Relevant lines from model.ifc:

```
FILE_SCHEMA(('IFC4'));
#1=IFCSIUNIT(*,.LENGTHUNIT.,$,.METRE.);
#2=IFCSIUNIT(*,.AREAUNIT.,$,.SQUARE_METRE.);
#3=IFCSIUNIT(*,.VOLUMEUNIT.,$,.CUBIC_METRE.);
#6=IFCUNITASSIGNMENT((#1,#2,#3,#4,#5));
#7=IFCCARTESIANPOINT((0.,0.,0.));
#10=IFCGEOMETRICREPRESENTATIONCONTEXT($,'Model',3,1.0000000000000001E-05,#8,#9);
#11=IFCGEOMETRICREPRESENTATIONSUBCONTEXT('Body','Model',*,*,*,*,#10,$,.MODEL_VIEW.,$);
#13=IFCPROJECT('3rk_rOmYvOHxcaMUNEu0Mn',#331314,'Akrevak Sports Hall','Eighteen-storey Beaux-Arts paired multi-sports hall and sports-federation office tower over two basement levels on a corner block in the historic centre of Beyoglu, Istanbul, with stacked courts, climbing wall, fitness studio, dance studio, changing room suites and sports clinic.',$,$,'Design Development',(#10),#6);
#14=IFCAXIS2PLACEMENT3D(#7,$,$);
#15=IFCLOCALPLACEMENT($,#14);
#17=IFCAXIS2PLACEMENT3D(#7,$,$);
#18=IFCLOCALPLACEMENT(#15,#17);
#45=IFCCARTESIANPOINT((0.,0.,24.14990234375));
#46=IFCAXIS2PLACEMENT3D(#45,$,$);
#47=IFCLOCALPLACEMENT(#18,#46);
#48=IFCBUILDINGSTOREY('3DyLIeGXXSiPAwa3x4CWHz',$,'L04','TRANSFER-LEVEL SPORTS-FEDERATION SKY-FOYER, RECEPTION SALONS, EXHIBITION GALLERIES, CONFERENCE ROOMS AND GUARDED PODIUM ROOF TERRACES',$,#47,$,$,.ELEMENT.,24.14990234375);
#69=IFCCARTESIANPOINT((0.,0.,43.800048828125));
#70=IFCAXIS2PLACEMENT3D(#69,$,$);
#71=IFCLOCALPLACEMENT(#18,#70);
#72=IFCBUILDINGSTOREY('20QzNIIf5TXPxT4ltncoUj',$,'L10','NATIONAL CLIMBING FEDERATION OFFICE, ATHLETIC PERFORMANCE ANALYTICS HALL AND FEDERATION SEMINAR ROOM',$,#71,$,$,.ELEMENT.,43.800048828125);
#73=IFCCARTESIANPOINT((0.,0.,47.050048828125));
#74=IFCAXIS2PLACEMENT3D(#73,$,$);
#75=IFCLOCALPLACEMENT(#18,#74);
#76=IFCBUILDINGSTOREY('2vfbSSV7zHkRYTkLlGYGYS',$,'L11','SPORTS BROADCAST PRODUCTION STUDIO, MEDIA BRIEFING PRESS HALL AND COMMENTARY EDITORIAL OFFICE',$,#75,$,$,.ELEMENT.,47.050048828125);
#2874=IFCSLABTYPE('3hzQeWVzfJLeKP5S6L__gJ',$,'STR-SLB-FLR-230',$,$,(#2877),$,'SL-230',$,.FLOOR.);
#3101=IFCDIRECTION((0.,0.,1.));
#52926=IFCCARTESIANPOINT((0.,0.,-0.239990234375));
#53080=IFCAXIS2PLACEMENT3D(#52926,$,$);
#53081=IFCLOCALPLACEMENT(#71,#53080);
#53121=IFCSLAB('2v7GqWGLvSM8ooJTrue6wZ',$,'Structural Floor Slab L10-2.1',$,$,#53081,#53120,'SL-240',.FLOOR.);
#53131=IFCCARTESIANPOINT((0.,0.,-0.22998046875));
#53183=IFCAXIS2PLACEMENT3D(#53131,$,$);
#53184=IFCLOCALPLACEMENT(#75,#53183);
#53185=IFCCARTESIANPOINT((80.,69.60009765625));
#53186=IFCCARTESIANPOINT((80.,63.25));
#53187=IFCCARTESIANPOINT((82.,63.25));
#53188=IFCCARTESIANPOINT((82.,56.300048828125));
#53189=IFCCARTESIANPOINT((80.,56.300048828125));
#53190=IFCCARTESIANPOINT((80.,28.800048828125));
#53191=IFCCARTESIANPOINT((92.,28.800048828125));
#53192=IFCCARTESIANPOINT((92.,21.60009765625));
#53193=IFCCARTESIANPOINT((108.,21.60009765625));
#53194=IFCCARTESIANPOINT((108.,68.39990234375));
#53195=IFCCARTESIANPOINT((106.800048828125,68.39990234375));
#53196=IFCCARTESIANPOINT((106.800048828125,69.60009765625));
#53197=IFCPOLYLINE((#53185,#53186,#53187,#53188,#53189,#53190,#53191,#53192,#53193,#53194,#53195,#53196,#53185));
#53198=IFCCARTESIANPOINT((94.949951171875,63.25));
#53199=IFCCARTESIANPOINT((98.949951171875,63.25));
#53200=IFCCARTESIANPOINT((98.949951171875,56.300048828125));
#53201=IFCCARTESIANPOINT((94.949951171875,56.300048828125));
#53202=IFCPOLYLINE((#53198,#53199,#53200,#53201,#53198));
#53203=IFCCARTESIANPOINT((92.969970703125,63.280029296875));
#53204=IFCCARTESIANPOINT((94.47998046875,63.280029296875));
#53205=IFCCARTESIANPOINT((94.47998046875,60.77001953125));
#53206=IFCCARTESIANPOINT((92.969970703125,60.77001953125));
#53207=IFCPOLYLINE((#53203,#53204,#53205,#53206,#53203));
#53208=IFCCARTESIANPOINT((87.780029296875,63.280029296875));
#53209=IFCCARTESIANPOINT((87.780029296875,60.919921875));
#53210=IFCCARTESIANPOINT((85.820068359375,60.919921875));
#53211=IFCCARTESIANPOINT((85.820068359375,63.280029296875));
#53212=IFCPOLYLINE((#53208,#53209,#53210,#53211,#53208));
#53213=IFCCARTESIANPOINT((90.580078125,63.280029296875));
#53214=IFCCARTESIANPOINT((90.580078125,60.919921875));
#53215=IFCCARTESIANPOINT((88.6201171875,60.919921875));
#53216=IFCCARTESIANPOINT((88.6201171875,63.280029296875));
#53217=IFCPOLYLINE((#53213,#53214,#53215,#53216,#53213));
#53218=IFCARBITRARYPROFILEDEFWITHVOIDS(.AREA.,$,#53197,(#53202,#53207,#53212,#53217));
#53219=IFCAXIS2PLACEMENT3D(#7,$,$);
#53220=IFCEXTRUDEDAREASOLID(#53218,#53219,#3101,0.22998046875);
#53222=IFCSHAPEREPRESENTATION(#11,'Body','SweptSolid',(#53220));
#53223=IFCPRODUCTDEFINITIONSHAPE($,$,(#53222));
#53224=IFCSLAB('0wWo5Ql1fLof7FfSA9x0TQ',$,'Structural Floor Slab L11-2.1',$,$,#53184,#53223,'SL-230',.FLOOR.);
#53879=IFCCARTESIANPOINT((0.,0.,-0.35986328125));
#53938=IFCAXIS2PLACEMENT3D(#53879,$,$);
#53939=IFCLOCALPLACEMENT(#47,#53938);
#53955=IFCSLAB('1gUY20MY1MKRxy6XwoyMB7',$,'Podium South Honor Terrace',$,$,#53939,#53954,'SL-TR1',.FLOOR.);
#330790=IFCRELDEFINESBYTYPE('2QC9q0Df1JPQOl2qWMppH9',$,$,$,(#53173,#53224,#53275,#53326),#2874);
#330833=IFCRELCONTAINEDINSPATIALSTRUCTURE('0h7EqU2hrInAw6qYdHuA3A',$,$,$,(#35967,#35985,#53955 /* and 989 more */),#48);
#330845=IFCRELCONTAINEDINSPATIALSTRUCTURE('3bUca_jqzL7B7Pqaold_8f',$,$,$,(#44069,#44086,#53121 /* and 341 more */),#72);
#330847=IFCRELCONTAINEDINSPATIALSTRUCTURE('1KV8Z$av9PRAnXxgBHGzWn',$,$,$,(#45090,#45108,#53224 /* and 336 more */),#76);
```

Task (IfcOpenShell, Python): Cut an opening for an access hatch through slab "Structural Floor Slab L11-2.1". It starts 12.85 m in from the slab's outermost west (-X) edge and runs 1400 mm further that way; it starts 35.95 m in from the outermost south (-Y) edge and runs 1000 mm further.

```python
import numpy as np
import ifcopenshell
import ifcopenshell.api.feature
import ifcopenshell.api.geometry
import ifcopenshell.api.root
import ifcopenshell.geom
import ifcopenshell.util.placement
import ifcopenshell.util.representation
import ifcopenshell.util.shape
import ifcopenshell.util.unit

model = ifcopenshell.open("model.ifc")
unit_scale = ifcopenshell.util.unit.calculate_unit_scale(model)
settings = ifcopenshell.geom.settings()


def volume(element):
    """Net volume in cubic metres, openings subtracted."""
    shape = ifcopenshell.geom.create_shape(settings, element)
    return ifcopenshell.util.shape.get_volume(shape.geometry)


slab = model.by_id(53224)
before = volume(slab)

# Extent in the slab's own axes, in metres. The edges named are its -X and -Y sides.
slab_shape = ifcopenshell.geom.create_shape(settings, slab)
vertices = ifcopenshell.util.shape.get_vertices(slab_shape.geometry)
x_min, y_min, bottom = vertices.min(axis=0)
top = vertices[:, 2].max()

opening = ifcopenshell.api.root.create_entity(model, ifc_class="IfcOpeningElement", name="Access hatch opening", predefined_type="OPENING")
context = ifcopenshell.util.representation.get_context(model, "Model", "Body", "MODEL_VIEW")
width, depth = 1.4, 1
outline = [(0.0, 0.0), (width, 0.0), (width, depth), (0.0, depth), (0.0, 0.0)]
# Overshoot both faces by 50 mm so the cut is clean.
shape = ifcopenshell.api.geometry.add_slab_representation(
    model, context=context, depth=top - bottom + 0.1, polyline=outline
)
ifcopenshell.api.geometry.assign_representation(model, product=opening, representation=shape)

matrix = ifcopenshell.util.placement.get_local_placement(slab.ObjectPlacement)
matrix[:, 3] = matrix @ np.append(np.array([x_min + 12.85, y_min + 35.95, bottom - 0.05]) / unit_scale, 1.0)
ifcopenshell.api.geometry.edit_object_placement(model, product=opening, matrix=matrix, is_si=False)
ifcopenshell.api.feature.add_feature(model, feature=opening, element=slab)

after = volume(slab)

print(f"slab volume {before:.3f} -> {after:.3f} m3")

model.write("model_v2.ifc")
```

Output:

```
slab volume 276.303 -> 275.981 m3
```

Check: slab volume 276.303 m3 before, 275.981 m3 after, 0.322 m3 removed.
